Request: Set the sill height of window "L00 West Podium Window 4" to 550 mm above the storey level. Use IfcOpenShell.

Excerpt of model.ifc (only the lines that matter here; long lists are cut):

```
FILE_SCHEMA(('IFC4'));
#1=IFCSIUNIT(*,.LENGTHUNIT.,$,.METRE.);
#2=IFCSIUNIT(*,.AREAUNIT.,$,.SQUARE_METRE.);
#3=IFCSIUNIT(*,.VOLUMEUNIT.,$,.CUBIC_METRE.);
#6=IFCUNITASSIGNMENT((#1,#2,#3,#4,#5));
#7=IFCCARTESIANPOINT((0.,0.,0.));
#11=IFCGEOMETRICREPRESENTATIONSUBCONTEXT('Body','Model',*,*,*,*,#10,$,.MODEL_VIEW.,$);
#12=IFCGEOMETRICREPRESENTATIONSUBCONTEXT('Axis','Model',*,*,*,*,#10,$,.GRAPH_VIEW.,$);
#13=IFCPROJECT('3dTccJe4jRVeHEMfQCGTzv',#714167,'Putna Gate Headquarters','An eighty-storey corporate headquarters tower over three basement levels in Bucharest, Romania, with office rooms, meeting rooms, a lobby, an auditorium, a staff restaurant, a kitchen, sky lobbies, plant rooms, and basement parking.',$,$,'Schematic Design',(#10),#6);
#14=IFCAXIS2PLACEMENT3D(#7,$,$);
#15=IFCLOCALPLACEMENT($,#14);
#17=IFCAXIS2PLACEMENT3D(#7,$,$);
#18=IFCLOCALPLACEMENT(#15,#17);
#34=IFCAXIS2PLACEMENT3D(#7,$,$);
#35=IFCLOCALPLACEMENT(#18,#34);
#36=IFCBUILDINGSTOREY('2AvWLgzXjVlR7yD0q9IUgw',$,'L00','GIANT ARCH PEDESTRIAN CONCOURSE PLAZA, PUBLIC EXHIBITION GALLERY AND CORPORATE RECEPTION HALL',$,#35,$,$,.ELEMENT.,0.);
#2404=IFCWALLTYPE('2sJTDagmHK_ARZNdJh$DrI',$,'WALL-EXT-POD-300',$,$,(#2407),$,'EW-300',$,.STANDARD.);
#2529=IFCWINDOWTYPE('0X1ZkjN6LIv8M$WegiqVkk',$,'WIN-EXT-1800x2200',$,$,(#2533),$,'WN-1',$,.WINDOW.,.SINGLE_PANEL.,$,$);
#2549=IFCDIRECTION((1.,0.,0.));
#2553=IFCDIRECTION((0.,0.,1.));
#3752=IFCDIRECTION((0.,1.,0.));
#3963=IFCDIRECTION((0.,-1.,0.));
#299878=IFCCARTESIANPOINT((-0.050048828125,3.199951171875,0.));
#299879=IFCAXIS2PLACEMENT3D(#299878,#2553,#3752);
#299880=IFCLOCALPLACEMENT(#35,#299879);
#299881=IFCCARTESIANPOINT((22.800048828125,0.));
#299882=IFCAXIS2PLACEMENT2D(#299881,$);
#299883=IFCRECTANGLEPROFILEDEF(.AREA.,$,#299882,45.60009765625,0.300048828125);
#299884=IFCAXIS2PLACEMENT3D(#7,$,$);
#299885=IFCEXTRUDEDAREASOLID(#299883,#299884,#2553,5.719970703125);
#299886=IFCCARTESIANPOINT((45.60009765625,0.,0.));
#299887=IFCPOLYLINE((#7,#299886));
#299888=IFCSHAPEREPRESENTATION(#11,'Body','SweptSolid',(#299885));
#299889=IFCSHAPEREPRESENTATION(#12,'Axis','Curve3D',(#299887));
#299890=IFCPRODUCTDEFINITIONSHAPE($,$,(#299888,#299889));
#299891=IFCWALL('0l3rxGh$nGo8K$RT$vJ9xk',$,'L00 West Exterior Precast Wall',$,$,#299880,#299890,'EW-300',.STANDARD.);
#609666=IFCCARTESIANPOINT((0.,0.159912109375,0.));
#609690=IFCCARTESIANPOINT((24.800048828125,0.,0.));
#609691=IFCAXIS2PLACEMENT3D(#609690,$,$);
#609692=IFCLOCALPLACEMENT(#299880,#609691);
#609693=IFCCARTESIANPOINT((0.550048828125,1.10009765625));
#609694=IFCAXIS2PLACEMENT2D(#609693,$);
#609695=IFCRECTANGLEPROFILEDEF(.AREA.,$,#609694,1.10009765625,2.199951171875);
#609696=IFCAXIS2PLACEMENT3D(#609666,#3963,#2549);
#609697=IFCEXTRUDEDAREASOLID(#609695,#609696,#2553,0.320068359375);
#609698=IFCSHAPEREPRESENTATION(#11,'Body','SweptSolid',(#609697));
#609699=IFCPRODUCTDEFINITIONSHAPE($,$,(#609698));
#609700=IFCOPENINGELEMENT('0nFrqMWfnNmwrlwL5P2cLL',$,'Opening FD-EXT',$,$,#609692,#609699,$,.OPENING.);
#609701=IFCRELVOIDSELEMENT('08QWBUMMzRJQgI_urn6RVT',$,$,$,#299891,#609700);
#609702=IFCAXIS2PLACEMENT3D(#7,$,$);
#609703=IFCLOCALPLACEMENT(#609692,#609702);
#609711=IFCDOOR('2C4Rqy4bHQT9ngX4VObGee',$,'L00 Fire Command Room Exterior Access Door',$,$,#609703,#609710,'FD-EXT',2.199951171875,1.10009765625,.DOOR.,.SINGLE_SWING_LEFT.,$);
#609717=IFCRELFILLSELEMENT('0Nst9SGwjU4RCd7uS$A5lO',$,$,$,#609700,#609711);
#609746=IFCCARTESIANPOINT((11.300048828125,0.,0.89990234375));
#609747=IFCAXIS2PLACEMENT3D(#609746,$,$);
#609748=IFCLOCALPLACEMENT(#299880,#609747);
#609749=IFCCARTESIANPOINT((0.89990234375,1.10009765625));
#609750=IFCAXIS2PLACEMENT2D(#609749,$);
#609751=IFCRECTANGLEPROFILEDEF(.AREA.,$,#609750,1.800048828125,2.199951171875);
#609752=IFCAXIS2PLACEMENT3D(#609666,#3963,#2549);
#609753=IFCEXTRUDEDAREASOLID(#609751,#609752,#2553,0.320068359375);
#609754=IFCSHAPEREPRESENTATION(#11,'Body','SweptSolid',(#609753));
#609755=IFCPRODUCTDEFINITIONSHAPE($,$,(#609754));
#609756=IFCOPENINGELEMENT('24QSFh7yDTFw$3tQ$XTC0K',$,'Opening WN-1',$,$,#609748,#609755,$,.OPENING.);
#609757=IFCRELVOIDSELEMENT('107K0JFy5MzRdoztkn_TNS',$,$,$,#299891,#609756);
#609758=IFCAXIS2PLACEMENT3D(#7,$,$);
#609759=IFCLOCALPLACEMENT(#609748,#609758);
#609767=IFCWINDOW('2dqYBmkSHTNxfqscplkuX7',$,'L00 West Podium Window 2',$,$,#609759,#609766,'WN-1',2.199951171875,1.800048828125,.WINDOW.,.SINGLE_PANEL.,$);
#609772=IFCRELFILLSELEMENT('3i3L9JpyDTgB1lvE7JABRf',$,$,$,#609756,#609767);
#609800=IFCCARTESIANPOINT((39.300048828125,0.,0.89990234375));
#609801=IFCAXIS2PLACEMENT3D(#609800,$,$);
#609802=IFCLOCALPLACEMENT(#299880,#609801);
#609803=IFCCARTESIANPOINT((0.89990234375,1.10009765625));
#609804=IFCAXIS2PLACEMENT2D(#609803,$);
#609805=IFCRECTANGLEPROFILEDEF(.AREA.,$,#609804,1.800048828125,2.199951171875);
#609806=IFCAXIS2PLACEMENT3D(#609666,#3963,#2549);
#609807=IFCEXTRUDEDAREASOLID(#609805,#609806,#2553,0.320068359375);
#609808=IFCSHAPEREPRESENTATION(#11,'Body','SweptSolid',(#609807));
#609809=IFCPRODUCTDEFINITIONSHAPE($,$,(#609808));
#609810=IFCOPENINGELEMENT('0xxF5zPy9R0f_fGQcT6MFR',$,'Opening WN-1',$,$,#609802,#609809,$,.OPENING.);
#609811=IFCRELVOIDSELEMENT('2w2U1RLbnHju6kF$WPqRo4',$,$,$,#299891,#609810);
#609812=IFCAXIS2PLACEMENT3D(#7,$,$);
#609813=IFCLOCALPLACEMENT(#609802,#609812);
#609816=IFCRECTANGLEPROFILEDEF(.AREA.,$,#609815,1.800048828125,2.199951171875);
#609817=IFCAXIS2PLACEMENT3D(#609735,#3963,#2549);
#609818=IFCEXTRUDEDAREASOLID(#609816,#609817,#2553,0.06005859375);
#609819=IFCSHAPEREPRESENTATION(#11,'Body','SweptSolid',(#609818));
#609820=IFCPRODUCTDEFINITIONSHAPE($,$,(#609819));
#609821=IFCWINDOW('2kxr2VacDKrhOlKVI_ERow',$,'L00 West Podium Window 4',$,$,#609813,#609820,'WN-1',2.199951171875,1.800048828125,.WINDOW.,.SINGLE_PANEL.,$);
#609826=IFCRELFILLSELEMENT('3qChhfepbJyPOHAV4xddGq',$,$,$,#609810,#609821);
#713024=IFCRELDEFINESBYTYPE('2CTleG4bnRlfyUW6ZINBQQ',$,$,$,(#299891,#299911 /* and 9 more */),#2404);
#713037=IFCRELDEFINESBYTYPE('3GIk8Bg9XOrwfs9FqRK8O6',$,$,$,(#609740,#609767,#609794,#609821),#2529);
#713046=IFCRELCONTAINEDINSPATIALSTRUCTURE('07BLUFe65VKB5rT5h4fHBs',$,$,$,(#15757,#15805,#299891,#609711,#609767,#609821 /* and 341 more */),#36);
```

```python
import numpy as np
import ifcopenshell
import ifcopenshell.api.geometry
import ifcopenshell.geom
import ifcopenshell.util.element
import ifcopenshell.util.placement
import ifcopenshell.util.shape
import ifcopenshell.util.unit

model = ifcopenshell.open("model.ifc")
unit_scale = ifcopenshell.util.unit.calculate_unit_scale(model)

window = model.by_guid("2kxr2VacDKrhOlKVI_ERow")
opening = window.FillsVoids[0].RelatingOpeningElement
storey = ifcopenshell.util.element.get_container(window, ifc_class="IfcBuildingStorey")
level = ifcopenshell.util.placement.get_local_placement(storey.ObjectPlacement)[2, 3]

# The opening's origin need not be at the sill, so measure its lowest point.
shape = ifcopenshell.geom.create_shape(ifcopenshell.geom.settings(), opening)
bottom = ifcopenshell.util.shape.get_shape_bottom_elevation(shape, shape.geometry) / unit_scale
dz = level + 0.55 / unit_scale - bottom

shift = np.array([0.0, 0.0, dz])
# The window is placed relative to its opening, so it follows when the opening moves.
matrix = ifcopenshell.util.placement.get_local_placement(opening.ObjectPlacement)
matrix[:3, 3] += shift
ifcopenshell.api.geometry.edit_object_placement(
    model, product=opening, matrix=matrix, is_si=False, should_transform_children=True
)

print(f"moved by {dz * unit_scale:+.3f} m")

model.write("model-out.ifc")
```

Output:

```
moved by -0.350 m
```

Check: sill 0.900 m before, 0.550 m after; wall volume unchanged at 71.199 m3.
